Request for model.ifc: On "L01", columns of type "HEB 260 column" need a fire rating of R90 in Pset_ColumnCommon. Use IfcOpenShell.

First a look at what the model holds.

```python
import ifcopenshell
import ifcopenshell.util.element

model = ifcopenshell.open("model.ifc")
print(model.schema)
storey = next(s for s in model.by_type("IfcBuildingStorey") if s.Name == "L01")
columns = [e for e in ifcopenshell.util.element.get_decomposition(storey) if e.is_a("IfcColumn")]
seen = {}
for e in columns:
    element_type = ifcopenshell.util.element.get_type(e)
    key = (element_type.Name if element_type != e and element_type else None, ifcopenshell.util.element.get_pset(e, "Pset_ColumnCommon", "FireRating"))
    seen[key] = seen.get(key, 0) + 1
for (name, value), count in sorted(seen.items(), key=str):
    print(count, "x", name, "|", value)
```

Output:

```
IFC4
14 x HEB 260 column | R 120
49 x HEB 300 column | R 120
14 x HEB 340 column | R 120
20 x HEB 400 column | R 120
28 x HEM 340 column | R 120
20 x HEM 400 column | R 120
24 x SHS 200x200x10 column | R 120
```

```python
import ifcopenshell
import ifcopenshell.api.pset
import ifcopenshell.util.element

model = ifcopenshell.open("model.ifc")

storey = next(s for s in model.by_type("IfcBuildingStorey") if s.Name == "L01")
columns = [e for e in ifcopenshell.util.element.get_decomposition(storey) if e.is_a("IfcColumn")]

count = 0
for e in columns:
    element_type = ifcopenshell.util.element.get_type(e)
    if element_type in (None, e) or element_type.Name != "HEB 260 column":
        continue
    # add_pset returns the element's existing set when there is one.
    pset = ifcopenshell.api.pset.add_pset(model, product=e, name="Pset_ColumnCommon")
    ifcopenshell.api.pset.edit_pset(model, pset=pset, properties={"FireRating": "R90"})
    count += 1

print(count, "columns updated")

model.write("model-out.ifc")
```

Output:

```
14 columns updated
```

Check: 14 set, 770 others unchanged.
